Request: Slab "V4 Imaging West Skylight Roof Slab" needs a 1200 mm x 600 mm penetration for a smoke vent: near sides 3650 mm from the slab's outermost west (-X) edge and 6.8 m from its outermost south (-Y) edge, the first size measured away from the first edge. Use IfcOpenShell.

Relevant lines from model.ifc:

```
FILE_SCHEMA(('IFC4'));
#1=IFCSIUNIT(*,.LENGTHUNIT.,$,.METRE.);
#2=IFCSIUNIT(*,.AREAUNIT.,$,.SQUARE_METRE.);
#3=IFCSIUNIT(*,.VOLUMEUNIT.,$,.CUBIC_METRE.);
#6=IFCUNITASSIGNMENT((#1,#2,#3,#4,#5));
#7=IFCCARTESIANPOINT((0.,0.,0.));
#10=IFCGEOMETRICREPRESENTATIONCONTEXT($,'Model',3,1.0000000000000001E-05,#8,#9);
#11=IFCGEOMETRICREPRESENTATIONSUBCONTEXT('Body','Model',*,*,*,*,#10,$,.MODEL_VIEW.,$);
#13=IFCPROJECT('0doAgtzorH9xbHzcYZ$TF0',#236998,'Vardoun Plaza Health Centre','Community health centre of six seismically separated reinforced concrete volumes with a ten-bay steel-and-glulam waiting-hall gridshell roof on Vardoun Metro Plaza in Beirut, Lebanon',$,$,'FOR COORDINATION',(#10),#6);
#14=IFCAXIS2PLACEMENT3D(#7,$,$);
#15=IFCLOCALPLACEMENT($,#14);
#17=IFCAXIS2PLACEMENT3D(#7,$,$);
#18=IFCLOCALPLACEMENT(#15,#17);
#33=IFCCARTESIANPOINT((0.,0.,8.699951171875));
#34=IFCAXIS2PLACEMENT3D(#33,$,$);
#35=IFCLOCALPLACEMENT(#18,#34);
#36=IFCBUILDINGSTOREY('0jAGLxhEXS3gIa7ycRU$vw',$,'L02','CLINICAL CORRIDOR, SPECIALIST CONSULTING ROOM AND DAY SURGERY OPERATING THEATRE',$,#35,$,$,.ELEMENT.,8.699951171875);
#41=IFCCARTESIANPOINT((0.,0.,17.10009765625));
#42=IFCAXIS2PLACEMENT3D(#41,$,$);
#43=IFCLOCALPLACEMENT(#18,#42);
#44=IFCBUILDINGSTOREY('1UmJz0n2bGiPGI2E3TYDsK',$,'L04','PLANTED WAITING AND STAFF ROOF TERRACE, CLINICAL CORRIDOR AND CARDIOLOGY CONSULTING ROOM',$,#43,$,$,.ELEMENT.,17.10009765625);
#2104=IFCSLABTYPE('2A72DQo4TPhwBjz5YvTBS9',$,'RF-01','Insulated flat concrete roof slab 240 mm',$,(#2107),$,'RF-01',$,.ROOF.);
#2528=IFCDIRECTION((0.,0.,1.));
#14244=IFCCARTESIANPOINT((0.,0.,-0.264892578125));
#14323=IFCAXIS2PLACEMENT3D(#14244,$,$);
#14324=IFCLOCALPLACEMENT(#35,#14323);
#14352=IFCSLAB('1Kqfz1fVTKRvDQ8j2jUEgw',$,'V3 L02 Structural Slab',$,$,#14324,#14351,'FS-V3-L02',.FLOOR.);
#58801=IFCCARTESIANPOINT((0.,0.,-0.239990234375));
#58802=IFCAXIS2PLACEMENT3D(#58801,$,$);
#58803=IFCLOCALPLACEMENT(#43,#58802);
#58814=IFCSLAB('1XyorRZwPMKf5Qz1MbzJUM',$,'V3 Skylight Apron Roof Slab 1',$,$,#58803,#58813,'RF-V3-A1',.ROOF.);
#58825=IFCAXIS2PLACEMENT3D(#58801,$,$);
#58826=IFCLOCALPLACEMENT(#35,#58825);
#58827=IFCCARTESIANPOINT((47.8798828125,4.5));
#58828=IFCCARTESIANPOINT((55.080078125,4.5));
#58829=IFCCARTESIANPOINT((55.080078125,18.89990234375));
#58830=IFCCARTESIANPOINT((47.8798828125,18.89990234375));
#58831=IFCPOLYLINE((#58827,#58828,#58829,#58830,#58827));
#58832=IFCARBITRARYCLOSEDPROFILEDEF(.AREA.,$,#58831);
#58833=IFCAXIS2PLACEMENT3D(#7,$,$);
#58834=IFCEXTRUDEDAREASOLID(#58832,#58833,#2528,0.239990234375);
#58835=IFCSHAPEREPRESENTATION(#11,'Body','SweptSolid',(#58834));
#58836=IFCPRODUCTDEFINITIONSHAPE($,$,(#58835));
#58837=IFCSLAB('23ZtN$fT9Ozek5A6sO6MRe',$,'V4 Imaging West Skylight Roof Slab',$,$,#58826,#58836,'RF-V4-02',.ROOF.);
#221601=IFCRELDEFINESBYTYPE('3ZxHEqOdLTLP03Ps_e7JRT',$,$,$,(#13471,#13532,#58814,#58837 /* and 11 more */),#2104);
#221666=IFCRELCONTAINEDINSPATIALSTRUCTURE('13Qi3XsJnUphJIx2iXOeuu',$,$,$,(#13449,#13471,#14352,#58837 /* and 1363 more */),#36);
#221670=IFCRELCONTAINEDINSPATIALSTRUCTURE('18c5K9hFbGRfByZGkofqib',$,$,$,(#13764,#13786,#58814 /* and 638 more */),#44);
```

```python
import numpy as np
import ifcopenshell
import ifcopenshell.api.feature
import ifcopenshell.api.geometry
import ifcopenshell.api.root
import ifcopenshell.geom
import ifcopenshell.util.placement
import ifcopenshell.util.representation
import ifcopenshell.util.shape
import ifcopenshell.util.unit

model = ifcopenshell.open("model.ifc")
unit_scale = ifcopenshell.util.unit.calculate_unit_scale(model)
settings = ifcopenshell.geom.settings()


def volume(element):
    """Net volume in cubic metres, openings subtracted."""
    shape = ifcopenshell.geom.create_shape(settings, element)
    return ifcopenshell.util.shape.get_volume(shape.geometry)


slab = model.by_guid("23ZtN$fT9Ozek5A6sO6MRe")
before = volume(slab)

# Extent in the slab's own axes, in metres. The edges named are its -X and -Y sides.
slab_shape = ifcopenshell.geom.create_shape(settings, slab)
vertices = ifcopenshell.util.shape.get_vertices(slab_shape.geometry)
x_min, y_min, bottom = vertices.min(axis=0)
top = vertices[:, 2].max()

opening = ifcopenshell.api.root.create_entity(model, ifc_class="IfcOpeningElement", name="Smoke vent opening", predefined_type="OPENING")
context = ifcopenshell.util.representation.get_context(model, "Model", "Body", "MODEL_VIEW")
width, depth = 1.2, 0.6
outline = [(0.0, 0.0), (width, 0.0), (width, depth), (0.0, depth), (0.0, 0.0)]
# Overshoot both faces by 50 mm so the cut is clean.
shape = ifcopenshell.api.geometry.add_slab_representation(
    model, context=context, depth=top - bottom + 0.1, polyline=outline
)
ifcopenshell.api.geometry.assign_representation(model, product=opening, representation=shape)

matrix = ifcopenshell.util.placement.get_local_placement(slab.ObjectPlacement)
matrix[:, 3] = matrix @ np.append(np.array([x_min + 3.65, y_min + 6.8, bottom - 0.05]) / unit_scale, 1.0)
ifcopenshell.api.geometry.edit_object_placement(model, product=opening, matrix=matrix, is_si=False)
ifcopenshell.api.feature.add_feature(model, feature=opening, element=slab)

after = volume(slab)

print(f"slab volume {before:.3f} -> {after:.3f} m3")

model.write("model_updated.ifc")
```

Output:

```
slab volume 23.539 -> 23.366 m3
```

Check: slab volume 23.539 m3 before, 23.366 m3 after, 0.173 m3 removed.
